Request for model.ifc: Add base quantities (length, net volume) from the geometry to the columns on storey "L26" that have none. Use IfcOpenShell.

First a look at what the model holds.

```python
import ifcopenshell
import ifcopenshell.util.element
import ifcopenshell.util.unit

model = ifcopenshell.open("model.ifc")
print(model.schema)
for unit_type in ("LENGTHUNIT", "AREAUNIT", "VOLUMEUNIT"):
    print(unit_type, ifcopenshell.util.unit.calculate_unit_scale(model, unit_type))
storey = next(s for s in model.by_type("IfcBuildingStorey") if s.Name == "L26")
columns = [e for e in ifcopenshell.util.element.get_decomposition(storey) if e.is_a("IfcColumn")]
for e in sorted(columns, key=lambda e: e.id()):
    print(e.id(), e.is_a(), e.Name, list(ifcopenshell.util.element.get_psets(e, qtos_only=True)), sep=" | ")
```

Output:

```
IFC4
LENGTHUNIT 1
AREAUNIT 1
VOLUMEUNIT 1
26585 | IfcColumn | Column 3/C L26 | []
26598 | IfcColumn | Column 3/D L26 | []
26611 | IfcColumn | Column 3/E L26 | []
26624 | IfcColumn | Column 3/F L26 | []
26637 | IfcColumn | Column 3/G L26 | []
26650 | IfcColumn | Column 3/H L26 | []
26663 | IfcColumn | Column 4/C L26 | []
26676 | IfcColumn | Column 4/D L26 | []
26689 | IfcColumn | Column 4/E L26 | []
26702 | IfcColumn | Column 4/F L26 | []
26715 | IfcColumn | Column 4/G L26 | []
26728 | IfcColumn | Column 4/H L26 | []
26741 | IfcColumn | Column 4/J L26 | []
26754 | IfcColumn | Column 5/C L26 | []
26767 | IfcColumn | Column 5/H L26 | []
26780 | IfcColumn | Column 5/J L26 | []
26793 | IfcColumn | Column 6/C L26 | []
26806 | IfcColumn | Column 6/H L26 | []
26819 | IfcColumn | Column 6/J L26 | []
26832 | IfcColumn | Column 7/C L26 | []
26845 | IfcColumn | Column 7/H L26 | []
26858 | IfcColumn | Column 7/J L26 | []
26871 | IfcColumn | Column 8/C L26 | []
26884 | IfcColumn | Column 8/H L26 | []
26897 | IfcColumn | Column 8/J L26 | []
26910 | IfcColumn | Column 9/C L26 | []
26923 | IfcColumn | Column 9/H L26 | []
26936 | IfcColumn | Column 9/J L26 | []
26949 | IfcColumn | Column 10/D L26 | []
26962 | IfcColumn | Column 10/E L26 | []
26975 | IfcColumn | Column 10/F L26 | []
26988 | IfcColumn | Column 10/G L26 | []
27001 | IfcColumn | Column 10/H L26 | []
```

```python
import ifcopenshell
import ifcopenshell.api.pset
import ifcopenshell.geom
import ifcopenshell.util.element
import ifcopenshell.util.shape
import ifcopenshell.util.unit

model = ifcopenshell.open("model.ifc")
unit_scale = ifcopenshell.util.unit.calculate_unit_scale(model)
volume_scale = ifcopenshell.util.unit.calculate_unit_scale(model, "VOLUMEUNIT")
settings = ifcopenshell.geom.settings()

storey = next(s for s in model.by_type("IfcBuildingStorey") if s.Name == "L26")
columns = [e for e in ifcopenshell.util.element.get_decomposition(storey) if e.is_a("IfcColumn")]

for e in sorted(columns, key=lambda e: e.id()):
    if ifcopenshell.util.element.get_psets(e, qtos_only=True, should_inherit=False):
        continue
    # Geometry comes back in metres, in the element's own axes.
    shape = ifcopenshell.geom.create_shape(settings, e)
    values = {
        "Length": ifcopenshell.util.shape.get_z(shape.geometry) / unit_scale,
        "NetVolume": ifcopenshell.util.shape.get_volume(shape.geometry) / volume_scale,
    }
    qto = ifcopenshell.api.pset.add_qto(model, product=e, name="Qto_ColumnBaseQuantities")
    ifcopenshell.api.pset.edit_qto(model, qto=qto, properties=values)
    print(e.id(), {k: round(v, 3) for k, v in values.items()})

model.write("model_v2.ifc")
```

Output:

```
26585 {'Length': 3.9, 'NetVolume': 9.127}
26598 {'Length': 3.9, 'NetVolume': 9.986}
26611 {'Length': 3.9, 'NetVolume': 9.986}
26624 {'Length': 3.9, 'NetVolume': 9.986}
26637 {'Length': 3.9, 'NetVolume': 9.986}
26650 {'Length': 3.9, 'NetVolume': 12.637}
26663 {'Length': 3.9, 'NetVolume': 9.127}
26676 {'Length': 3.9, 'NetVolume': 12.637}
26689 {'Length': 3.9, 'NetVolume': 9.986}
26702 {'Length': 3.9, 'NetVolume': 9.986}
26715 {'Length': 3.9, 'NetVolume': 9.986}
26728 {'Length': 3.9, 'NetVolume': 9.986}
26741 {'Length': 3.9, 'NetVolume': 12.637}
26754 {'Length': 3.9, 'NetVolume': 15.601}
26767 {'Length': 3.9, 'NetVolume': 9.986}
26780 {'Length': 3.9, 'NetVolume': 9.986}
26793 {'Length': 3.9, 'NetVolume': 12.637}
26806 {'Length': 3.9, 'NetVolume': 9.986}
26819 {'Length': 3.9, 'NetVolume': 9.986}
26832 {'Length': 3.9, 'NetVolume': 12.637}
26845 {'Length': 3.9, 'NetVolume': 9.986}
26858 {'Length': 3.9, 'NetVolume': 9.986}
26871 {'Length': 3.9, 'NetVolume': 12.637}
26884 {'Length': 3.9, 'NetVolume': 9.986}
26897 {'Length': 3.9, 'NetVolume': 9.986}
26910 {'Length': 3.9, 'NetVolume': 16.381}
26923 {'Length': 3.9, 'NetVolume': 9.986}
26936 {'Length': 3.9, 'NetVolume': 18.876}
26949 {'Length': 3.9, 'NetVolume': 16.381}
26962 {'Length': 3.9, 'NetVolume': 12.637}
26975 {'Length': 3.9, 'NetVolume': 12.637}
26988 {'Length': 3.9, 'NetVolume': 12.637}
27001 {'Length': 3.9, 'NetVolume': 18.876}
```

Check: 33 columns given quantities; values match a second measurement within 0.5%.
